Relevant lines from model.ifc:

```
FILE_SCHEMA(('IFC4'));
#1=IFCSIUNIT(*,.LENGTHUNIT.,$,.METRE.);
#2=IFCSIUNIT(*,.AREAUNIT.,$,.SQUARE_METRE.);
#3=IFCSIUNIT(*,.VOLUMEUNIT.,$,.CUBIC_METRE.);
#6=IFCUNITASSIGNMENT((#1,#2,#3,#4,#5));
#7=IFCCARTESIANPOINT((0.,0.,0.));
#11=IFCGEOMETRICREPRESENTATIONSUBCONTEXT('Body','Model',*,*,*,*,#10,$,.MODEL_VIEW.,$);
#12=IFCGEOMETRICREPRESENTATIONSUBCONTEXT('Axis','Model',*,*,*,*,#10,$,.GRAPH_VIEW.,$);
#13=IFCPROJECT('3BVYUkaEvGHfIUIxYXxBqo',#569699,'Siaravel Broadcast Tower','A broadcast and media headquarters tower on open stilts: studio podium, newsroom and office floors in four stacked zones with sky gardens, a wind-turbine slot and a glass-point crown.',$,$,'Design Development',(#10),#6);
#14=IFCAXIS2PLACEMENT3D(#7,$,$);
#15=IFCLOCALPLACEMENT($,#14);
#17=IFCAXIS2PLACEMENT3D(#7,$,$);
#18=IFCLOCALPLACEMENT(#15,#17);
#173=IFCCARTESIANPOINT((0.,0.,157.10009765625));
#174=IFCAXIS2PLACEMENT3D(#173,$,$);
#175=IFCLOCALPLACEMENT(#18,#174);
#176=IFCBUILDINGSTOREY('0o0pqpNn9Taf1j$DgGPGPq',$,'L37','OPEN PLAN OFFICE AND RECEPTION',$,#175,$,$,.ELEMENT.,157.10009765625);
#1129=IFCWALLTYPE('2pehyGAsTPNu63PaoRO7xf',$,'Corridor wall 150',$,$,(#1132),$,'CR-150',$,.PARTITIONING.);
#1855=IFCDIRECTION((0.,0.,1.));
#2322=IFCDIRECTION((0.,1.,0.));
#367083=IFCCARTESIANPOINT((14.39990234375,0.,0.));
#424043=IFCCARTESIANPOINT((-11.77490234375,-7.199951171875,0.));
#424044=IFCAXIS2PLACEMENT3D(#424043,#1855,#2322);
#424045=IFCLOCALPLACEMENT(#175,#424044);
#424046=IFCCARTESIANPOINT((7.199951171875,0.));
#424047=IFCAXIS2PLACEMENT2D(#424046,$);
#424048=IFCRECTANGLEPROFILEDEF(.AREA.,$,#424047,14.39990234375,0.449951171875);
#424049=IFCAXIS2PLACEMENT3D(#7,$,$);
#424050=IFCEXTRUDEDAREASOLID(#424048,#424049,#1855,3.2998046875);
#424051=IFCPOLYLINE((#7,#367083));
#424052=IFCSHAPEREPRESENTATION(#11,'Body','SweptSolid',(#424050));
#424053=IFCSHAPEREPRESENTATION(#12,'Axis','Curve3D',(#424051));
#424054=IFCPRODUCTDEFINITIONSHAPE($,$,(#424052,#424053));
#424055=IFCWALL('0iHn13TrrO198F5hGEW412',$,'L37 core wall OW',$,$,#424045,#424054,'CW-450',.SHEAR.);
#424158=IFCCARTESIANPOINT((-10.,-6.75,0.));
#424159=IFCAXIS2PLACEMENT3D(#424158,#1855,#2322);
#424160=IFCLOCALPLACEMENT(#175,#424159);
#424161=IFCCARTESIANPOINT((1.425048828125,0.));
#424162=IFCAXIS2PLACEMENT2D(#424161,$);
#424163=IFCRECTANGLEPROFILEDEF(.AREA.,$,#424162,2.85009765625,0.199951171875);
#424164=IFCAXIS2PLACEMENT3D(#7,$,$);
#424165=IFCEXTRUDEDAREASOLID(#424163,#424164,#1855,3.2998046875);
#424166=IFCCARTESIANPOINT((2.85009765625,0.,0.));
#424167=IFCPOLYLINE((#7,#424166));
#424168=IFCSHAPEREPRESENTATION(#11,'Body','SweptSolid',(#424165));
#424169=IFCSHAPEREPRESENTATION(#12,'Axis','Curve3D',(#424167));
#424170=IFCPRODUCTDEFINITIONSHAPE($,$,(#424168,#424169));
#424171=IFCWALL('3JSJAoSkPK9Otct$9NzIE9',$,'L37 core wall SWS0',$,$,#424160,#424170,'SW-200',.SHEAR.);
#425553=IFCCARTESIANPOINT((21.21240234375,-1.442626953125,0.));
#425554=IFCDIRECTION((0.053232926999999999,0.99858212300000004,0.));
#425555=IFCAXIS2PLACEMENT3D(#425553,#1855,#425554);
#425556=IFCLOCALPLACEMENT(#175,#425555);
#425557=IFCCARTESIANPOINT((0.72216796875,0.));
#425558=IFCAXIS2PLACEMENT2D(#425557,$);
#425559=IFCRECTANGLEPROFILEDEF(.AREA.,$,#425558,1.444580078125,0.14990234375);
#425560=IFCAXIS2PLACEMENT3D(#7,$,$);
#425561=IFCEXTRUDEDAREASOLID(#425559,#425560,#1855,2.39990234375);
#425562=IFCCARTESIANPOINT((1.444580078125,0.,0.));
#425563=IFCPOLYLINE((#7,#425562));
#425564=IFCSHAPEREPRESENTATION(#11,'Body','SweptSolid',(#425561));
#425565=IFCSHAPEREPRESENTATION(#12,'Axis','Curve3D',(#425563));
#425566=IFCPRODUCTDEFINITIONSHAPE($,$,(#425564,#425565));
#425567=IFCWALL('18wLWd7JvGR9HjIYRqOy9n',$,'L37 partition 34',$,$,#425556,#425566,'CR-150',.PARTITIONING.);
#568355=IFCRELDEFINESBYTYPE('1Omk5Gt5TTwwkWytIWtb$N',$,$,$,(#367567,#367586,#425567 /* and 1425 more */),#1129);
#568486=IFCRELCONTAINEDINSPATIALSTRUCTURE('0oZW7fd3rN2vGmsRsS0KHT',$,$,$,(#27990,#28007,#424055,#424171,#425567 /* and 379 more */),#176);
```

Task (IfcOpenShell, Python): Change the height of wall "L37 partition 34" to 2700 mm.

```python
import ifcopenshell
import ifcopenshell.geom
import ifcopenshell.util.representation
import ifcopenshell.util.shape

model = ifcopenshell.open("model.ifc")
settings = ifcopenshell.geom.settings()


def volume(element):
    """Net volume in cubic metres, openings subtracted."""
    shape = ifcopenshell.geom.create_shape(settings, element)
    return ifcopenshell.util.shape.get_volume(shape.geometry)


wall = model.by_id(425567)
before = volume(wall)

body = ifcopenshell.util.representation.get_representation(wall, "Model", "Body")
solid = body.Items[0]
old_height = solid.Depth
solid.Depth = 2.7
after = volume(wall)

print(f"height {old_height:g} -> {solid.Depth:g}, volume {before:.3f} -> {after:.3f} m3")

model.write("model_updated.ifc")
```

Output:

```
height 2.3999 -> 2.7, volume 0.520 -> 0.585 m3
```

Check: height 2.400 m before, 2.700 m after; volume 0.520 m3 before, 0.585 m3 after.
